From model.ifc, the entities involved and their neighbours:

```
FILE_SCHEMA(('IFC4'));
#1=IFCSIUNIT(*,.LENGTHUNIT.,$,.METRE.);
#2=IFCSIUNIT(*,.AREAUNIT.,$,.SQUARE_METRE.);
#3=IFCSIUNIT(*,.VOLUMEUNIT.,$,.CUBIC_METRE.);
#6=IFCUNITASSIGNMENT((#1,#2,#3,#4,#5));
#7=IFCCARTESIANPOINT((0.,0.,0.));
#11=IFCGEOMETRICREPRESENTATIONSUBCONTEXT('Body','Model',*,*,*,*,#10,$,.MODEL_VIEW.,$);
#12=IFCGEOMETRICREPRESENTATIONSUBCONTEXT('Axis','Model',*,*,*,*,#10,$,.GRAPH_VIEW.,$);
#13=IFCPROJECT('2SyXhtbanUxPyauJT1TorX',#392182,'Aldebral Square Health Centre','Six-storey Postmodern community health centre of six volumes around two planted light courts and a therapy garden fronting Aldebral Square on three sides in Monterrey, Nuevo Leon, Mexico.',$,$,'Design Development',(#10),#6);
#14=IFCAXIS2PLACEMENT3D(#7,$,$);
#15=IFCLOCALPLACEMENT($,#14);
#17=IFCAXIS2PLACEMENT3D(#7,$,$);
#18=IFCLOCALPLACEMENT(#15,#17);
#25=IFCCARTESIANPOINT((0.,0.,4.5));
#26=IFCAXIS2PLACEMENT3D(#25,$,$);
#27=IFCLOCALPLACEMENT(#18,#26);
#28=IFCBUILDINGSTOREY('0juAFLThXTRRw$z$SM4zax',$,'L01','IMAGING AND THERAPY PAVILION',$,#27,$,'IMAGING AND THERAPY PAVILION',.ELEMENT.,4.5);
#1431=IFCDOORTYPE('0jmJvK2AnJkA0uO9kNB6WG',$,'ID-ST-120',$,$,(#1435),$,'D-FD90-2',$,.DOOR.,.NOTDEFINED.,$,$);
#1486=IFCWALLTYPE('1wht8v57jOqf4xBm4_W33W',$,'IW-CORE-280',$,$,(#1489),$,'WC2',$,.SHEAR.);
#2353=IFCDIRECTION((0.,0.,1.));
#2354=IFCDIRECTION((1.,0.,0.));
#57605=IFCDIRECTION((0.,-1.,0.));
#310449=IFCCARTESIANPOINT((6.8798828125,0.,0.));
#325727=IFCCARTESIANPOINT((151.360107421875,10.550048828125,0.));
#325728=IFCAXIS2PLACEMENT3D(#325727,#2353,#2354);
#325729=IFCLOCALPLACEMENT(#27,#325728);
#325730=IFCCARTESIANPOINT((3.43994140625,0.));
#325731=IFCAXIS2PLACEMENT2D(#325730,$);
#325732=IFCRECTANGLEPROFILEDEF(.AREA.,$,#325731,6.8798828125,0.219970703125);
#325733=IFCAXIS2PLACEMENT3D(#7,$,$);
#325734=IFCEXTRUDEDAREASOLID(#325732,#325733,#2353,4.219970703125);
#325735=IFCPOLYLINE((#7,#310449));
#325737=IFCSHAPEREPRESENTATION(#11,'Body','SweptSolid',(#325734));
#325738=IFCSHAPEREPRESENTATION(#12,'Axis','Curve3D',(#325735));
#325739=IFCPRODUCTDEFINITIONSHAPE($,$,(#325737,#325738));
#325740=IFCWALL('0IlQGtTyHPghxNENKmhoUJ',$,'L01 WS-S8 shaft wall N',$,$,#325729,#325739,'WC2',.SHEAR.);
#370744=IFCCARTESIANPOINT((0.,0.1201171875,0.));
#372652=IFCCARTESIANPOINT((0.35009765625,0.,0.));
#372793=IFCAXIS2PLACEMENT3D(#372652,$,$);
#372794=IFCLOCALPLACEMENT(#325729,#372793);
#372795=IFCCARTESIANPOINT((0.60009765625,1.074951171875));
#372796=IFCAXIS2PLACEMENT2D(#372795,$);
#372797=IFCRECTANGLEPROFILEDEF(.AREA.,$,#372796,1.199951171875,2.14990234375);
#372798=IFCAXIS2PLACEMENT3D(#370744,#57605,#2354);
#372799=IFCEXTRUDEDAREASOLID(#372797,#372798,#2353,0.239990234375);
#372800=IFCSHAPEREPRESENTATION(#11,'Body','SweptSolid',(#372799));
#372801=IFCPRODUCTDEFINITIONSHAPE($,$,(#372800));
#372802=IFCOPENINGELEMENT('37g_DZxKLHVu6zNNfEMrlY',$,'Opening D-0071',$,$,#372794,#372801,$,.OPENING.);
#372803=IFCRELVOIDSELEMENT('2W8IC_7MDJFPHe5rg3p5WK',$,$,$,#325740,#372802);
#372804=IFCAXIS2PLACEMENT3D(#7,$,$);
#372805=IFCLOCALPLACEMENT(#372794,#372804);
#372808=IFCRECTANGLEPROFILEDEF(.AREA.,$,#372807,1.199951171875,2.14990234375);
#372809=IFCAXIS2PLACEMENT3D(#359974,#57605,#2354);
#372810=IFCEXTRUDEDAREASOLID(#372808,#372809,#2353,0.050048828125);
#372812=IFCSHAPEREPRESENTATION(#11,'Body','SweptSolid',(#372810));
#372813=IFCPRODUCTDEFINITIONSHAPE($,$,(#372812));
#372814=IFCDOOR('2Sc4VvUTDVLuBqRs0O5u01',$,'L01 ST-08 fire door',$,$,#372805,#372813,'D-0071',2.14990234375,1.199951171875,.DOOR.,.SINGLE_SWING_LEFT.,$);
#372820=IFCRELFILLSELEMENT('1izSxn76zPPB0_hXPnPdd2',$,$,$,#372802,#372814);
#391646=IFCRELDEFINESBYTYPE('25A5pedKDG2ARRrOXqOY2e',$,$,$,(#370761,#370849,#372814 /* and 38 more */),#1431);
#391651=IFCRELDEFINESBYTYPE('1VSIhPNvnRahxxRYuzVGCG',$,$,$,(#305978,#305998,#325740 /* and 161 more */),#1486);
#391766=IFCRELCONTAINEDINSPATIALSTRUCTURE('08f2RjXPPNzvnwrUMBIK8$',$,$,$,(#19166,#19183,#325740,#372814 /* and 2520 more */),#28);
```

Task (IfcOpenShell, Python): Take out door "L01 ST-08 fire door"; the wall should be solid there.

```python
import ifcopenshell
import ifcopenshell.api.feature
import ifcopenshell.api.root
import ifcopenshell.geom
import ifcopenshell.util.shape

model = ifcopenshell.open("model.ifc")
settings = ifcopenshell.geom.settings()


def volume(element):
    """Net volume in cubic metres, openings subtracted."""
    shape = ifcopenshell.geom.create_shape(settings, element)
    return ifcopenshell.util.shape.get_volume(shape.geometry)


door = model.by_id(372814)
opening = door.FillsVoids[0].RelatingOpeningElement
wall = opening.VoidsElements[0].RelatingBuildingElement
before = volume(wall)

ifcopenshell.api.root.remove_product(model, product=door)
ifcopenshell.api.feature.remove_feature(model, feature=opening)

after = volume(wall)

print(f"wall volume {before:.3f} -> {after:.3f} m3")

model.write("model_updated.ifc")
```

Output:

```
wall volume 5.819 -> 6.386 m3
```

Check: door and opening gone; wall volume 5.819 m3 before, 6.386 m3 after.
